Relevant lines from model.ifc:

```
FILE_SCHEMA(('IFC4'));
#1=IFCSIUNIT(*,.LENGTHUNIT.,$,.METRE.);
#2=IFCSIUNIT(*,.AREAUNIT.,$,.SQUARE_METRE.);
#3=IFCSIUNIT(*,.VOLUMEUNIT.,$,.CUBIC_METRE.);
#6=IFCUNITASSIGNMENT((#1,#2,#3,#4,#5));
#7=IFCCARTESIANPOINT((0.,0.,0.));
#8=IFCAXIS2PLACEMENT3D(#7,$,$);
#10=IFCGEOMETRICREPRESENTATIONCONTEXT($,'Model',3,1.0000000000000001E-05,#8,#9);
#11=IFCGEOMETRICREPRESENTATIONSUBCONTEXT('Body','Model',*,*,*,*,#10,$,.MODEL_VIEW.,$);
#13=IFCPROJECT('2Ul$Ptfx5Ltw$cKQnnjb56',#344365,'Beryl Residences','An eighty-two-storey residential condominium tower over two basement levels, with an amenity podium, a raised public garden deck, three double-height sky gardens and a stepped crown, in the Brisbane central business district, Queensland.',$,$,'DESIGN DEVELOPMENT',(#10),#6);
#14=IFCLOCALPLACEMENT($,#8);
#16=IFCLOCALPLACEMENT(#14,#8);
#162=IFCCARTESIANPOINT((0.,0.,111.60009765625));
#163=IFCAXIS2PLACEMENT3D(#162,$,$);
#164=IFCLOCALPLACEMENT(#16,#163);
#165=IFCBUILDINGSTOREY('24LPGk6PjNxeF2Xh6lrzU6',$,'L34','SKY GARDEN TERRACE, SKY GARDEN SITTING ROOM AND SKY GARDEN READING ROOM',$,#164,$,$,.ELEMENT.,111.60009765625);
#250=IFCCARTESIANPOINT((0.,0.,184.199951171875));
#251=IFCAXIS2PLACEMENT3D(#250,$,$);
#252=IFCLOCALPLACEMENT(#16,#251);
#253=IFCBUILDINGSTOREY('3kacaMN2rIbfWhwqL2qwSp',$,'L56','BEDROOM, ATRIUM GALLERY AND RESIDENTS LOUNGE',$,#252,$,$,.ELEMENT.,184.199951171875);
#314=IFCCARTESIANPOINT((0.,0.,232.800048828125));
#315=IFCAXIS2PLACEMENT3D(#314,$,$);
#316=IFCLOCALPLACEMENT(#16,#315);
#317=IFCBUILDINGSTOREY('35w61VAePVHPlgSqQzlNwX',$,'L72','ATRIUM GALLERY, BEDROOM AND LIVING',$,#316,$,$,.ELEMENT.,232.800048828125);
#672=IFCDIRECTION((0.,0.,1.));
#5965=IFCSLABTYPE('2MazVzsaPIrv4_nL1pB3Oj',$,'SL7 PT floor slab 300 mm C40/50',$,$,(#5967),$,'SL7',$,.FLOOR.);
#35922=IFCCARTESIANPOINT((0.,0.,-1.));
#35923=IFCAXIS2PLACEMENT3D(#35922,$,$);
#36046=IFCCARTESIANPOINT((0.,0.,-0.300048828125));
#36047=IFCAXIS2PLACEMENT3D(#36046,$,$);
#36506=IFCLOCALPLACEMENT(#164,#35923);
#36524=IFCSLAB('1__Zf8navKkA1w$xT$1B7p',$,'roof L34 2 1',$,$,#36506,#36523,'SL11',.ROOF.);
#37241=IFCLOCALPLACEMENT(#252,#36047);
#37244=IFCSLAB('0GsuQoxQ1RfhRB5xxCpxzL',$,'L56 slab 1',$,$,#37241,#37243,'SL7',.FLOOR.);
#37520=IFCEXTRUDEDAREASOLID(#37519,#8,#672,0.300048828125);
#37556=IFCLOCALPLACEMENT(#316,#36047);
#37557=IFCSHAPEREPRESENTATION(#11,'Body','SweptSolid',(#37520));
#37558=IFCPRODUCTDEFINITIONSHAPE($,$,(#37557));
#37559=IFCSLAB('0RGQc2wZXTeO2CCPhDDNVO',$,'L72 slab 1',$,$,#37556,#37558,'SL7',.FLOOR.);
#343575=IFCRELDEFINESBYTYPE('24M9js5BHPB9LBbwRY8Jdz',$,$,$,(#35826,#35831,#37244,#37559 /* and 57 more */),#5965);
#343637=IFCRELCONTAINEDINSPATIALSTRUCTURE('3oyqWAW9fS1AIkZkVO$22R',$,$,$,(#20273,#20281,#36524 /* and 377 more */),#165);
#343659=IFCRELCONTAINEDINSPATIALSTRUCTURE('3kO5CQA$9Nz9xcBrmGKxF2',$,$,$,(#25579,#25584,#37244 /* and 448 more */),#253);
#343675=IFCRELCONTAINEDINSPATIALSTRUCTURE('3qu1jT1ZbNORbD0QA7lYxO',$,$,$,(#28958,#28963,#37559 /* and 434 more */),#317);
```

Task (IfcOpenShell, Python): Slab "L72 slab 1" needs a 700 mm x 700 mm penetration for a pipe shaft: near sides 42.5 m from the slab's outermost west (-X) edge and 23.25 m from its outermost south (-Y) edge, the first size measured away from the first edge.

```python
import numpy as np
import ifcopenshell
import ifcopenshell.api.feature
import ifcopenshell.api.geometry
import ifcopenshell.api.root
import ifcopenshell.geom
import ifcopenshell.util.placement
import ifcopenshell.util.representation
import ifcopenshell.util.shape
import ifcopenshell.util.unit

model = ifcopenshell.open("model.ifc")
unit_scale = ifcopenshell.util.unit.calculate_unit_scale(model)
settings = ifcopenshell.geom.settings()


def volume(element):
    """Net volume in cubic metres, openings subtracted."""
    shape = ifcopenshell.geom.create_shape(settings, element)
    return ifcopenshell.util.shape.get_volume(shape.geometry)


slab = model.by_id(37559)
before = volume(slab)

# Extent in the slab's own axes, in metres. The edges named are its -X and -Y sides.
slab_shape = ifcopenshell.geom.create_shape(settings, slab)
vertices = ifcopenshell.util.shape.get_vertices(slab_shape.geometry)
x_min, y_min, bottom = vertices.min(axis=0)
top = vertices[:, 2].max()

opening = ifcopenshell.api.root.create_entity(model, ifc_class="IfcOpeningElement", name="Pipe shaft opening", predefined_type="OPENING")
context = ifcopenshell.util.representation.get_context(model, "Model", "Body", "MODEL_VIEW")
width, depth = 0.7, 0.7
outline = [(0.0, 0.0), (width, 0.0), (width, depth), (0.0, depth), (0.0, 0.0)]
# Overshoot both faces by 50 mm so the cut is clean.
shape = ifcopenshell.api.geometry.add_slab_representation(
    model, context=context, depth=top - bottom + 0.1, polyline=outline
)
ifcopenshell.api.geometry.assign_representation(model, product=opening, representation=shape)

matrix = ifcopenshell.util.placement.get_local_placement(slab.ObjectPlacement)
matrix[:, 3] = matrix @ np.append(np.array([x_min + 42.5, y_min + 23.25, bottom - 0.05]) / unit_scale, 1.0)
ifcopenshell.api.geometry.edit_object_placement(model, product=opening, matrix=matrix, is_si=False)
ifcopenshell.api.feature.add_feature(model, feature=opening, element=slab)

after = volume(slab)

print(f"slab volume {before:.3f} -> {after:.3f} m3")

model.write("model_rev.ifc")
```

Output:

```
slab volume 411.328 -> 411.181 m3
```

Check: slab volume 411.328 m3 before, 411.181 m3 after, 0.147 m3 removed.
